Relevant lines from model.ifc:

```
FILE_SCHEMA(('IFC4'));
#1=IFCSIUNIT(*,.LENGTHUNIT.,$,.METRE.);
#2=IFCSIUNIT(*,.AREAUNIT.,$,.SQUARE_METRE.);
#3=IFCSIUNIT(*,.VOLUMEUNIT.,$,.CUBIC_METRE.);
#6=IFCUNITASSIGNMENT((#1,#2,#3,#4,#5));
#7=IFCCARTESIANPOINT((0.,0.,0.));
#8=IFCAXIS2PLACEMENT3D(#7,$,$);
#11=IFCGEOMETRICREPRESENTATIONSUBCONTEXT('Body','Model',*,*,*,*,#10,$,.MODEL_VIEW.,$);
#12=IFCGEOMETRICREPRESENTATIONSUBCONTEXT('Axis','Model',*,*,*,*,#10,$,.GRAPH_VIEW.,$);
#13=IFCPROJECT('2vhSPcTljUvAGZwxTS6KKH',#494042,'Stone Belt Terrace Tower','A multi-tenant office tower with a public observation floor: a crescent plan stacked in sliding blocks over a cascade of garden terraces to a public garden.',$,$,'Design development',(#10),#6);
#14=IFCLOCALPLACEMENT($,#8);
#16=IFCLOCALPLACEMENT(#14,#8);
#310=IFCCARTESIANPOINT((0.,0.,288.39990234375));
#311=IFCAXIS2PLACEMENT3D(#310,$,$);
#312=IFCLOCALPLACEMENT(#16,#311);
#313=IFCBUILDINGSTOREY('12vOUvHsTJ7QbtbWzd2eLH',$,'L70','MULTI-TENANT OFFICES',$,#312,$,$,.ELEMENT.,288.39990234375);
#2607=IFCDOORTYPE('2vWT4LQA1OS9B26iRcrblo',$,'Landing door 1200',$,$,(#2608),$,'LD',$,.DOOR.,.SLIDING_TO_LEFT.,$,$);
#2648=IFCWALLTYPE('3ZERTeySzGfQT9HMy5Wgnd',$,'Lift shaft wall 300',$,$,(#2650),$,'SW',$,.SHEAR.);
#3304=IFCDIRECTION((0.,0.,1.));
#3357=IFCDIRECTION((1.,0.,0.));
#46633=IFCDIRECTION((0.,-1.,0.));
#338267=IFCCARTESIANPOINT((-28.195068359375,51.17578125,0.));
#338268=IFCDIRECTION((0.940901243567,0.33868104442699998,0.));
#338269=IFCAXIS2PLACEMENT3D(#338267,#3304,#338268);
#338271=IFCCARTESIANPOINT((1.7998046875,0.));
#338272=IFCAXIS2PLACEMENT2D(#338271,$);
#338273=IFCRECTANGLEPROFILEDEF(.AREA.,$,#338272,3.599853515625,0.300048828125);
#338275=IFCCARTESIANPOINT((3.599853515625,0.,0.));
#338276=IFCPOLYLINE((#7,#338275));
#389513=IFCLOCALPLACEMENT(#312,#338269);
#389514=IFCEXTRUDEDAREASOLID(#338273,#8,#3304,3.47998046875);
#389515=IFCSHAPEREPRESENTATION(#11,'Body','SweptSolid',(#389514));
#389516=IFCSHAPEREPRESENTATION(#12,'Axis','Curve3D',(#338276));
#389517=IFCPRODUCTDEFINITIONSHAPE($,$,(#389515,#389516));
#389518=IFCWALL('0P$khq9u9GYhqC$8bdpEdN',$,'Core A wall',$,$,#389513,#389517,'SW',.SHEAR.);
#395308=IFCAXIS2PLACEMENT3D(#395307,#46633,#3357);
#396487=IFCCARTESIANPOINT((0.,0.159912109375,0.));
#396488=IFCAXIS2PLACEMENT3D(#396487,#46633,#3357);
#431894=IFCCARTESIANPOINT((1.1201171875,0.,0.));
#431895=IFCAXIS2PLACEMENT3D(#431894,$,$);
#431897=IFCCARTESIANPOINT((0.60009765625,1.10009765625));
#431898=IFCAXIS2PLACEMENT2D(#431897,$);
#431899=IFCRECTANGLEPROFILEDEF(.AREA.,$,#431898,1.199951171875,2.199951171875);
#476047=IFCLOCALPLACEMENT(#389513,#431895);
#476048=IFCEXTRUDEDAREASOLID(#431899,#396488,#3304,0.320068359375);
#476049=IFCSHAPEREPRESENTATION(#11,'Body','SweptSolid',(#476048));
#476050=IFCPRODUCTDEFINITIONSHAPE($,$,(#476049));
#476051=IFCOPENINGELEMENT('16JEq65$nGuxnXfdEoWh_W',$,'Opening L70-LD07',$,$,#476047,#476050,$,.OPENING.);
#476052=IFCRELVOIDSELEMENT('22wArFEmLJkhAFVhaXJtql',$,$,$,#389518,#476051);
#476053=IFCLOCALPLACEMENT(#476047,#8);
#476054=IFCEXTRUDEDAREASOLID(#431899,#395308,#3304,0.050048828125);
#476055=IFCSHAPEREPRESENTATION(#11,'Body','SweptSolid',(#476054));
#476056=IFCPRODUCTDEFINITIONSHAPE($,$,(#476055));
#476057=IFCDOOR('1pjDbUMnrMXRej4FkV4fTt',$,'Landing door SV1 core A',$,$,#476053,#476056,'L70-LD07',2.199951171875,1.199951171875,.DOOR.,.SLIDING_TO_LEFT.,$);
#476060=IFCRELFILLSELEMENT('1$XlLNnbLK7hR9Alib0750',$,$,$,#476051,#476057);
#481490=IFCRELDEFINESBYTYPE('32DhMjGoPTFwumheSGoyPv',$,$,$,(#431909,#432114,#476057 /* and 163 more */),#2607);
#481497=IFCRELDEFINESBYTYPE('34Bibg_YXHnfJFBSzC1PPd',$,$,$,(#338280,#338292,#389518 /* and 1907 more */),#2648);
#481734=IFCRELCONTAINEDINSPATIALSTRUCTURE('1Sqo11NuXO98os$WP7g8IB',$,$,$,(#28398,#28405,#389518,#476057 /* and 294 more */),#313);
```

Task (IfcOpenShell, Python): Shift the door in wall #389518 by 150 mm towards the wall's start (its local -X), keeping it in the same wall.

```python
import ifcopenshell
import ifcopenshell.api.geometry
import ifcopenshell.util.placement

model = ifcopenshell.open("model.ifc")

door = model.by_guid("1pjDbUMnrMXRej4FkV4fTt")
opening = door.FillsVoids[0].RelatingOpeningElement
wall = opening.VoidsElements[0].RelatingBuildingElement

wall_matrix = ifcopenshell.util.placement.get_local_placement(wall.ObjectPlacement)
shift = wall_matrix[:3, 0] * -0.15
before = ifcopenshell.util.placement.get_local_placement(door.ObjectPlacement)[:3, 3].copy()

# The door is placed relative to its opening, so it follows when the opening moves.
matrix = ifcopenshell.util.placement.get_local_placement(opening.ObjectPlacement)
matrix[:3, 3] += shift
ifcopenshell.api.geometry.edit_object_placement(
    model, product=opening, matrix=matrix, is_si=False, should_transform_children=True
)

after = ifcopenshell.util.placement.get_local_placement(door.ObjectPlacement)[:3, 3]
print("door moved by", (after - before).round(3) + 0.0)

model.write("model_updated.ifc")
```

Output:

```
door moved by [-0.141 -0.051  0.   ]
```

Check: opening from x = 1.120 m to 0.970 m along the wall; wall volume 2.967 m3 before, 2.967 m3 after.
